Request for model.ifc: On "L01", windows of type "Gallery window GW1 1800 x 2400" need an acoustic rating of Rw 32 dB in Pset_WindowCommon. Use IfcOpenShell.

First a look at what the model holds.

```python
import ifcopenshell
import ifcopenshell.util.element

model = ifcopenshell.open("model.ifc")
print(model.schema)
storey = next(s for s in model.by_type("IfcBuildingStorey") if s.Name == "L01")
windows = [e for e in ifcopenshell.util.element.get_decomposition(storey) if e.is_a("IfcWindow")]
seen = {}
for e in windows:
    element_type = ifcopenshell.util.element.get_type(e)
    key = (element_type.Name if element_type != e and element_type else None, ifcopenshell.util.element.get_pset(e, "Pset_WindowCommon", "AcousticRating"))
    seen[key] = seen.get(key, 0) + 1
for (name, value), count in sorted(seen.items(), key=str):
    print(count, "x", name, "|", value)
```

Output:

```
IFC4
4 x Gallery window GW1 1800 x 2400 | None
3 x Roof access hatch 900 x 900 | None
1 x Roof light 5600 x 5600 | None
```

```python
import ifcopenshell
import ifcopenshell.api.pset
import ifcopenshell.util.element

model = ifcopenshell.open("model.ifc")

storey = next(s for s in model.by_type("IfcBuildingStorey") if s.Name == "L01")
windows = [e for e in ifcopenshell.util.element.get_decomposition(storey) if e.is_a("IfcWindow")]

count = 0
for e in windows:
    element_type = ifcopenshell.util.element.get_type(e)
    if element_type in (None, e) or element_type.Name != "Gallery window GW1 1800 x 2400":
        continue
    # add_pset returns the element's existing set when there is one.
    pset = ifcopenshell.api.pset.add_pset(model, product=e, name="Pset_WindowCommon")
    ifcopenshell.api.pset.edit_pset(model, pset=pset, properties={"AcousticRating": "Rw 32 dB"})
    count += 1

print(count, "windows updated")

model.write("model_updated.ifc")
```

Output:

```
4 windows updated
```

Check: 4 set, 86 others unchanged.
